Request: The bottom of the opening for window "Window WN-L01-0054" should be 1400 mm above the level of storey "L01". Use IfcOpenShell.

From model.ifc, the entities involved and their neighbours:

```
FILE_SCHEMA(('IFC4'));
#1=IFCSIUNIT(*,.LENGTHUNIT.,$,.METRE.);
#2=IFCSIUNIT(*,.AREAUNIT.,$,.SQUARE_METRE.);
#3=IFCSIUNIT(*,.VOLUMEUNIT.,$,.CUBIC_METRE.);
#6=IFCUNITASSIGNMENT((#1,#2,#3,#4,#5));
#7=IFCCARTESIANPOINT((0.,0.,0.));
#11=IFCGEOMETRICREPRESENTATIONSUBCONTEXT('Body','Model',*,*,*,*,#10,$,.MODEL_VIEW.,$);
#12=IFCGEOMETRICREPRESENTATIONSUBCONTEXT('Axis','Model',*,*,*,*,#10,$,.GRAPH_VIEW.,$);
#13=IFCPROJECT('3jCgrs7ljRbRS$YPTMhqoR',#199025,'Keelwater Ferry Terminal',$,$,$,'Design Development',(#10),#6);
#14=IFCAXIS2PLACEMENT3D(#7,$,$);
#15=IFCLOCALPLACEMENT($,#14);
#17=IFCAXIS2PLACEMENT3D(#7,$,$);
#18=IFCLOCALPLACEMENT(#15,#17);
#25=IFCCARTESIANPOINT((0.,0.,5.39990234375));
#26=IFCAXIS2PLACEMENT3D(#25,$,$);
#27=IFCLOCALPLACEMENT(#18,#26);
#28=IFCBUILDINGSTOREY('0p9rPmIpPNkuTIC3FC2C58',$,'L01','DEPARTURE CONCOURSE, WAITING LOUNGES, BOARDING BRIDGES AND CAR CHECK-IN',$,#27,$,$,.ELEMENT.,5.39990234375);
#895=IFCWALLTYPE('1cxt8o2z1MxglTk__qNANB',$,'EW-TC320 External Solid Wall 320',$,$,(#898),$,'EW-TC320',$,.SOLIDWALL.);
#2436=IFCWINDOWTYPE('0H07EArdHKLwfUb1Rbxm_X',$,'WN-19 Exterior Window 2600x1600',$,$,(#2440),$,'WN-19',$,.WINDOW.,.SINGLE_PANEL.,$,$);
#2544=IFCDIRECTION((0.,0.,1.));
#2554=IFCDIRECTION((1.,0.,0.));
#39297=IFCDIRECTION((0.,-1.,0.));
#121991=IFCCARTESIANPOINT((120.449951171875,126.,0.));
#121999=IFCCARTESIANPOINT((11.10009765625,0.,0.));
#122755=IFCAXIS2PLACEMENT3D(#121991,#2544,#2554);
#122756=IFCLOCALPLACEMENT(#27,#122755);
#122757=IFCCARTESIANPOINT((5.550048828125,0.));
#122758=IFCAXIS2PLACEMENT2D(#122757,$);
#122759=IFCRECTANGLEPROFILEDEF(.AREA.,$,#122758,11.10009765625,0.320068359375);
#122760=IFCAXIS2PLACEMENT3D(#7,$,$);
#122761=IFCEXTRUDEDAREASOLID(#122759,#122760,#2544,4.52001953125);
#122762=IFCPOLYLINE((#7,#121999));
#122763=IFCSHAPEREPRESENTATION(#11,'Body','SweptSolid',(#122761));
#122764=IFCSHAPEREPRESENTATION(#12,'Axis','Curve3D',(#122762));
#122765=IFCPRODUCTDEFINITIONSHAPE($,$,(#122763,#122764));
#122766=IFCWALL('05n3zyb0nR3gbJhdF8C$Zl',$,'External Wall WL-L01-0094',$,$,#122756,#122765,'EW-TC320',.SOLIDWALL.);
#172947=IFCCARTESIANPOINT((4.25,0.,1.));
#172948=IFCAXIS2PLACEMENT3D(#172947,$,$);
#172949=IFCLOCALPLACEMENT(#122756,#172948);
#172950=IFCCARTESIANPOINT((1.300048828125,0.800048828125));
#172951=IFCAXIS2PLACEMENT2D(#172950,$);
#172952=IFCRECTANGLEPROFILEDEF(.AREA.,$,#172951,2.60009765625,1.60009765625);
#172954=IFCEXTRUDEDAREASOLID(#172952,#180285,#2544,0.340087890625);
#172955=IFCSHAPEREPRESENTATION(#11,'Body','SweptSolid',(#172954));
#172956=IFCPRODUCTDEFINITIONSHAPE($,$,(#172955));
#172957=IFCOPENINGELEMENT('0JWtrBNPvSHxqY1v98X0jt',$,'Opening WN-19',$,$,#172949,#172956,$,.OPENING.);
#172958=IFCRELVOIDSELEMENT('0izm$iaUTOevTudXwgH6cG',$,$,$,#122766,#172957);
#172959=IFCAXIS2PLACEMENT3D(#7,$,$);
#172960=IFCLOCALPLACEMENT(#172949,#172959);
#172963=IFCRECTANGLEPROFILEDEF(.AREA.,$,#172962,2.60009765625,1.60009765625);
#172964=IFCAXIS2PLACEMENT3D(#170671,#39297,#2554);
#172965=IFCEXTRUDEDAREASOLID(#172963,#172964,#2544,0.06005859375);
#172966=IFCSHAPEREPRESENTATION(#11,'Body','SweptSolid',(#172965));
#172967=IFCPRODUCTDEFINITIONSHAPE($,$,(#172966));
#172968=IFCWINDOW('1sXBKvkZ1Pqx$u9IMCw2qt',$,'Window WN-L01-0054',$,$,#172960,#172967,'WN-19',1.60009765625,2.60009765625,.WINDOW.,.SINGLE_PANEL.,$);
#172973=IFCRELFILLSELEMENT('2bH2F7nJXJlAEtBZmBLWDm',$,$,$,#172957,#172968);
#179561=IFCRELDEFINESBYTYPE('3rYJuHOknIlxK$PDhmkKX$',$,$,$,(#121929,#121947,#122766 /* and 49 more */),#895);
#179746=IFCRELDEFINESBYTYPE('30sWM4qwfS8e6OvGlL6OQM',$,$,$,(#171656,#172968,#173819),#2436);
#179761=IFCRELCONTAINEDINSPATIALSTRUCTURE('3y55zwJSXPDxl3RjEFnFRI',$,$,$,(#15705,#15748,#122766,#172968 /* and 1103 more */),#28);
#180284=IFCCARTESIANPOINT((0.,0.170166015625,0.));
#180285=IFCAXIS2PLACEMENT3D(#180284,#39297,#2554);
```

```python
import numpy as np
import ifcopenshell
import ifcopenshell.api.geometry
import ifcopenshell.geom
import ifcopenshell.util.element
import ifcopenshell.util.placement
import ifcopenshell.util.shape
import ifcopenshell.util.unit

model = ifcopenshell.open("model.ifc")
unit_scale = ifcopenshell.util.unit.calculate_unit_scale(model)

window = model.by_guid("1sXBKvkZ1Pqx$u9IMCw2qt")
opening = window.FillsVoids[0].RelatingOpeningElement
storey = ifcopenshell.util.element.get_container(window, ifc_class="IfcBuildingStorey")
level = ifcopenshell.util.placement.get_local_placement(storey.ObjectPlacement)[2, 3]

# The opening's origin need not be at the sill, so measure its lowest point.
shape = ifcopenshell.geom.create_shape(ifcopenshell.geom.settings(), opening)
bottom = ifcopenshell.util.shape.get_shape_bottom_elevation(shape, shape.geometry) / unit_scale
dz = level + 1.4 / unit_scale - bottom

shift = np.array([0.0, 0.0, dz])
# The window is placed relative to its opening, so it follows when the opening moves.
matrix = ifcopenshell.util.placement.get_local_placement(opening.ObjectPlacement)
matrix[:3, 3] += shift
ifcopenshell.api.geometry.edit_object_placement(
    model, product=opening, matrix=matrix, is_si=False, should_transform_children=True
)

print(f"moved by {dz * unit_scale:+.3f} m")

model.write("model_rev.ifc")
```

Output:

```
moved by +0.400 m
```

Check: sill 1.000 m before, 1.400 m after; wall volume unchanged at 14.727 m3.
